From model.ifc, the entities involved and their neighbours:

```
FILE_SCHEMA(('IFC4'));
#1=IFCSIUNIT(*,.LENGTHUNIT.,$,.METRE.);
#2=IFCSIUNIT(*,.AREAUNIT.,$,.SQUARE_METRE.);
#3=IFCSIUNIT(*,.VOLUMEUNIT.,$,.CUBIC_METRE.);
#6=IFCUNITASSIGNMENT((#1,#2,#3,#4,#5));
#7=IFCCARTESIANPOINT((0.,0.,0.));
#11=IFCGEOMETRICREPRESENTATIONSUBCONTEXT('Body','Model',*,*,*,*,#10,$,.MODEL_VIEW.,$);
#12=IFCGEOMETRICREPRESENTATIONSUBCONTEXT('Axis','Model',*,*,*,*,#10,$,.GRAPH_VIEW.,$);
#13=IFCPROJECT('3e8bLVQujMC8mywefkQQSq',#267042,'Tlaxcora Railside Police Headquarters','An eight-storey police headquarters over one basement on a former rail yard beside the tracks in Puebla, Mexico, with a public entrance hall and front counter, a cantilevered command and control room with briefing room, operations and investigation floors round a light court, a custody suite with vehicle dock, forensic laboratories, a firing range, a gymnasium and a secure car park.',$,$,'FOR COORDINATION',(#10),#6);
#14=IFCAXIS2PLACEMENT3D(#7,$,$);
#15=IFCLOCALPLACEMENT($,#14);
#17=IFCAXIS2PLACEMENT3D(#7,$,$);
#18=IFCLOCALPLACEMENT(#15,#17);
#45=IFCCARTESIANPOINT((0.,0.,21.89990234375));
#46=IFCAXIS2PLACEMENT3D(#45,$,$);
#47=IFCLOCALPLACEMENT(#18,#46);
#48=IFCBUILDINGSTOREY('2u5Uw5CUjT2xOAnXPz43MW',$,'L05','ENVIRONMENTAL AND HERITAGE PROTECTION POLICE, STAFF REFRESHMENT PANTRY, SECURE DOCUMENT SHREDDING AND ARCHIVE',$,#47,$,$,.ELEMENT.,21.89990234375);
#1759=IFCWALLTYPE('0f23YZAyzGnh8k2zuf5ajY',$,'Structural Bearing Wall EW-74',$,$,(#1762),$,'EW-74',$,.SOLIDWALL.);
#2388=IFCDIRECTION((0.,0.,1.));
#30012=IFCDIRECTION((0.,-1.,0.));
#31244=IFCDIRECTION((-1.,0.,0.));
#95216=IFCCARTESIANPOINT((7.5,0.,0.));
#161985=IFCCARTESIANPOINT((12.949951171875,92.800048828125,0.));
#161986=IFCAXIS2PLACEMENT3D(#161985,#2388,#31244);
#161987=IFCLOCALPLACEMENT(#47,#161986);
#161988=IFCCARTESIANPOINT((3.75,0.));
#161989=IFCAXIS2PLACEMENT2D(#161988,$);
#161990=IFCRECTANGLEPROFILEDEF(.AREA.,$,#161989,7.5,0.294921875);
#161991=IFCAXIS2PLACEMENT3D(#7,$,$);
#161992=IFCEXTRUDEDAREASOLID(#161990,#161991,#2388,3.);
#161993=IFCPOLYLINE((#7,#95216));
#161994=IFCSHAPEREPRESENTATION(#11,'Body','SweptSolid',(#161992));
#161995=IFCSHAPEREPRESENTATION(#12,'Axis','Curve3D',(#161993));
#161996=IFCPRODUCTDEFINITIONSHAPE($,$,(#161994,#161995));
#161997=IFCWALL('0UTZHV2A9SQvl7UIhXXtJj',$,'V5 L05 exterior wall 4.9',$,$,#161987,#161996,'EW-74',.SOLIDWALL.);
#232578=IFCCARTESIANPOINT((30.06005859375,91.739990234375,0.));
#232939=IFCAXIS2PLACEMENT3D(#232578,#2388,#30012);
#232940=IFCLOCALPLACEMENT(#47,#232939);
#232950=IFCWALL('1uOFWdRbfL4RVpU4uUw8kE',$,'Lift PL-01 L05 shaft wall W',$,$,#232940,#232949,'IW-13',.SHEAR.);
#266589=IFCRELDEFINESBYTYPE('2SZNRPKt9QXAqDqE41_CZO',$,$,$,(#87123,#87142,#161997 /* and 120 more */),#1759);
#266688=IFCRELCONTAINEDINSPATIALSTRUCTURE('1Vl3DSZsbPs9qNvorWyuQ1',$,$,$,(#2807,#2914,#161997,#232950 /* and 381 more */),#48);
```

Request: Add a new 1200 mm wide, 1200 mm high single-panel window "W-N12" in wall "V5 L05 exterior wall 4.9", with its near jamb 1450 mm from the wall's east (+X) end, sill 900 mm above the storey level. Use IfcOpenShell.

```python
import numpy as np
import ifcopenshell
import ifcopenshell.api.feature
import ifcopenshell.api.geometry
import ifcopenshell.api.root
import ifcopenshell.api.spatial
import ifcopenshell.geom
import ifcopenshell.util.element
import ifcopenshell.util.placement
import ifcopenshell.util.representation
import ifcopenshell.util.shape
import ifcopenshell.util.unit

model = ifcopenshell.open("model.ifc")
unit_scale = ifcopenshell.util.unit.calculate_unit_scale(model)
settings = ifcopenshell.geom.settings()


def volume(element):
    """Net volume in cubic metres, openings subtracted."""
    shape = ifcopenshell.geom.create_shape(settings, element)
    return ifcopenshell.util.shape.get_volume(shape.geometry)


wall = model.by_guid("0UTZHV2A9SQvl7UIhXXtJj")
storey = ifcopenshell.util.element.get_container(wall, ifc_class="IfcBuildingStorey")
context = ifcopenshell.util.representation.get_context(model, "Model", "Body", "MODEL_VIEW")
before = volume(wall)

width, height, from_end, sill = 1.2, 1.2, 1.45, 0.9  # metres

# The wall runs along its own X axis, and the end named is its -X end.
wall_shape = ifcopenshell.geom.create_shape(settings, wall)
x, y, z = ifcopenshell.util.shape.get_vertices(wall_shape.geometry).T
start = x.min() + from_end
face, thickness = float(y.min()), float(y.max() - y.min())
wall_matrix = ifcopenshell.util.placement.get_local_placement(wall.ObjectPlacement)
level = ifcopenshell.util.placement.get_local_placement(storey.ObjectPlacement)[2, 3]


def in_wall(x, y):
    """Placement at x, y metres in the wall's axes, at sill height."""
    matrix = wall_matrix.copy()
    matrix[:, 3] = wall_matrix @ np.array([x / unit_scale, y / unit_scale, 0.0, 1.0])
    matrix[2, 3] = level + sill / unit_scale
    return matrix


# Opening: a box that overshoots both wall faces by 50 mm.
opening = ifcopenshell.api.root.create_entity(model, ifc_class="IfcOpeningElement", predefined_type="OPENING")
box = ifcopenshell.api.geometry.add_wall_representation(
    model, context=context, length=width, height=height, thickness=thickness + 0.1
)
ifcopenshell.api.geometry.assign_representation(model, product=opening, representation=box)
ifcopenshell.api.geometry.edit_object_placement(model, product=opening, matrix=in_wall(start, face - 0.05), is_si=False)
ifcopenshell.api.feature.add_feature(model, feature=opening, element=wall)

window = ifcopenshell.api.root.create_entity(model, ifc_class="IfcWindow", name="W-N12", predefined_type="WINDOW")
window.OverallWidth, window.OverallHeight = width / unit_scale, height / unit_scale
window.PartitioningType = "SINGLE_PANEL"
body = ifcopenshell.api.geometry.add_window_representation(
    model,
    context=context,
    overall_width=window.OverallWidth,
    overall_height=window.OverallHeight,
    partition_type="SINGLE_PANEL",
)
ifcopenshell.api.geometry.assign_representation(model, product=window, representation=body)
ifcopenshell.api.spatial.assign_container(model, products=[window], relating_structure=storey)
ifcopenshell.api.feature.add_filling(model, opening=opening, element=window)

# Centre the window in the wall's thickness.
ifcopenshell.api.geometry.edit_object_placement(model, product=window, matrix=in_wall(start, face), is_si=False)
window_shape = ifcopenshell.geom.create_shape(settings, window)
depth = ifcopenshell.util.shape.get_vertices(window_shape.geometry)[:, 1]
offset = face + thickness / 2 - (depth.min() + depth.max()) / 2
ifcopenshell.api.geometry.edit_object_placement(model, product=window, matrix=in_wall(start, offset), is_si=False)

after = volume(wall)

print(f"wall volume {before:.3f} -> {after:.3f} m3")

model.write("model_edited.ifc")
```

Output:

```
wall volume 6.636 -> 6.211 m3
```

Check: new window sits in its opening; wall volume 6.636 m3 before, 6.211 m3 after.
